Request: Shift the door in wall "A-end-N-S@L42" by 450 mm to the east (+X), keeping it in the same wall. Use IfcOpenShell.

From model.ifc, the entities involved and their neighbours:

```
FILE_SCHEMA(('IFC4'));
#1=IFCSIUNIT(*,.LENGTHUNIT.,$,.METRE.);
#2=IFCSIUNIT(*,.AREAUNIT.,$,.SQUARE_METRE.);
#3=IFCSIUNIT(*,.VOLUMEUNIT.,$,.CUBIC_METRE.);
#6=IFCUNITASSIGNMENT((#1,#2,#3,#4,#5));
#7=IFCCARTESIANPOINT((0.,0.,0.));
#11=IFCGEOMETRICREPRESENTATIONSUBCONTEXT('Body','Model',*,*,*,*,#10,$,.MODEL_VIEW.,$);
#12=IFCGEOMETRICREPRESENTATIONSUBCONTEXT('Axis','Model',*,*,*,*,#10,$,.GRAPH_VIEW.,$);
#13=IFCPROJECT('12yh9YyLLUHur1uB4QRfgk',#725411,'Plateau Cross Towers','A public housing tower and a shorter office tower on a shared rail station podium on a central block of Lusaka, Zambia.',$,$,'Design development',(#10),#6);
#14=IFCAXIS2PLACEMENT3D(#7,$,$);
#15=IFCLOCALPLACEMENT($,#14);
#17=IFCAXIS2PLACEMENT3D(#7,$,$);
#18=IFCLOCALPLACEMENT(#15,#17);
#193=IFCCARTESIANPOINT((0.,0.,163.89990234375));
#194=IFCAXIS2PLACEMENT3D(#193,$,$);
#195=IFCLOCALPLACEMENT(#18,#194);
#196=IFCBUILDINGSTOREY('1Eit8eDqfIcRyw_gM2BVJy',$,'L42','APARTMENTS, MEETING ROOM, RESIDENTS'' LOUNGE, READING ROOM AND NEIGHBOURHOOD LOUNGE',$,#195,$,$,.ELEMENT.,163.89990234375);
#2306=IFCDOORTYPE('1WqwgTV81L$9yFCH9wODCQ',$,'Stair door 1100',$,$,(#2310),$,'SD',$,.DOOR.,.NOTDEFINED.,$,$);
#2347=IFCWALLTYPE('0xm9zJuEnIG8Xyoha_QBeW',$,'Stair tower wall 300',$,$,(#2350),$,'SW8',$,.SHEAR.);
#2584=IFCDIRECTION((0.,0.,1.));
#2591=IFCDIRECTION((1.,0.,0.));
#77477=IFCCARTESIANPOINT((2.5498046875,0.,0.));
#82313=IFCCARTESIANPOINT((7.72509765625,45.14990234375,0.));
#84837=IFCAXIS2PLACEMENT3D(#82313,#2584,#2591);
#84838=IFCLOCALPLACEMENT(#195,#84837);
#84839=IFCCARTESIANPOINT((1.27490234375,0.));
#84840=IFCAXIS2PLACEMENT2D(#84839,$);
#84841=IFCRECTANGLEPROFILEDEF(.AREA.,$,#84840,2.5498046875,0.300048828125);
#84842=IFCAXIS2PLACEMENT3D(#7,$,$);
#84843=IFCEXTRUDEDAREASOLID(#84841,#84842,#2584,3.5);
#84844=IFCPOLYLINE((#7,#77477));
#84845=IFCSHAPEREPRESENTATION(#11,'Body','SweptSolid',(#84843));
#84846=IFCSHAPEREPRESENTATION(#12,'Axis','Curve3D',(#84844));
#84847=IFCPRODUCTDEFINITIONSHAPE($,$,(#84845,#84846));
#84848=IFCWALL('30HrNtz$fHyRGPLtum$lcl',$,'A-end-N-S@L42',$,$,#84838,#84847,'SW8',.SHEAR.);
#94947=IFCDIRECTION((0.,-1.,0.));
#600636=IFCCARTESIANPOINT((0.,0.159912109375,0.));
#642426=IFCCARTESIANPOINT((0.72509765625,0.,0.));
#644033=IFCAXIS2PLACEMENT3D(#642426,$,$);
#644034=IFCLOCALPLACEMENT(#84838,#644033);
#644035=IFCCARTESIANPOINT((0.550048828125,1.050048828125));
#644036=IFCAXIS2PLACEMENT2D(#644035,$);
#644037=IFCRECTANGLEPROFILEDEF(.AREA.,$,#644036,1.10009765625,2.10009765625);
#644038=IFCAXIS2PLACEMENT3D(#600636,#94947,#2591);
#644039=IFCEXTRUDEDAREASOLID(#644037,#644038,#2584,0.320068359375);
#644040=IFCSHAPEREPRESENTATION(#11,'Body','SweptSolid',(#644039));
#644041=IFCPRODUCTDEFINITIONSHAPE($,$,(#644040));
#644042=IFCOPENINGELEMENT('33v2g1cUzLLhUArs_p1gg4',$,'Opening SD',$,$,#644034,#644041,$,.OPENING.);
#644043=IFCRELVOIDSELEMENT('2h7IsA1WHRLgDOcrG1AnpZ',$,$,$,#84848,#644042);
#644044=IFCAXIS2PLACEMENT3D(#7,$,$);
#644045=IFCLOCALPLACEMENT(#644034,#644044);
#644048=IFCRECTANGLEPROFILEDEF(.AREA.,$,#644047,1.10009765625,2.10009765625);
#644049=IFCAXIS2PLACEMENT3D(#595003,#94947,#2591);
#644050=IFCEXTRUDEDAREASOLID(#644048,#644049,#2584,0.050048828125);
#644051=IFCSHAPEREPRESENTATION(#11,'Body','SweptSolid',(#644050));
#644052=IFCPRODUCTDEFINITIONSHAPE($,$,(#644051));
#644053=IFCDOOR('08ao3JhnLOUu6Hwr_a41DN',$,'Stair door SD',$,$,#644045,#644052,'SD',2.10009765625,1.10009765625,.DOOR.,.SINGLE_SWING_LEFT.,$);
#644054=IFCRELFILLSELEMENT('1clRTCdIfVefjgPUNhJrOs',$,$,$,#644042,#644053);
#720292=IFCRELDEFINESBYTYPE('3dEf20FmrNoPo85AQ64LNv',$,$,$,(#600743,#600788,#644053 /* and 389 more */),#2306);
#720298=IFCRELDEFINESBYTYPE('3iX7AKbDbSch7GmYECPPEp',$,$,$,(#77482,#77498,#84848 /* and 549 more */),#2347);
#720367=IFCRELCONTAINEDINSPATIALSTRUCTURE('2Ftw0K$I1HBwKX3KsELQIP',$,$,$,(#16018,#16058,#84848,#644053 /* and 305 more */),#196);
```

```python
import ifcopenshell
import ifcopenshell.api.geometry
import ifcopenshell.util.placement
import ifcopenshell.util.unit

model = ifcopenshell.open("model.ifc")
unit_scale = ifcopenshell.util.unit.calculate_unit_scale(model)

door = model.by_guid("08ao3JhnLOUu6Hwr_a41DN")
opening = door.FillsVoids[0].RelatingOpeningElement
wall = opening.VoidsElements[0].RelatingBuildingElement

wall_matrix = ifcopenshell.util.placement.get_local_placement(wall.ObjectPlacement)
shift = wall_matrix[:3, 0] * 0.45 / unit_scale
before = ifcopenshell.util.placement.get_local_placement(door.ObjectPlacement)[:3, 3].copy()

# The door is placed relative to its opening, so it follows when the opening moves.
matrix = ifcopenshell.util.placement.get_local_placement(opening.ObjectPlacement)
matrix[:3, 3] += shift
ifcopenshell.api.geometry.edit_object_placement(
    model, product=opening, matrix=matrix, is_si=False, should_transform_children=True
)

after = ifcopenshell.util.placement.get_local_placement(door.ObjectPlacement)[:3, 3]
print("door moved by", (after - before).round(3) + 0.0)

model.write("model_updated.ifc")
```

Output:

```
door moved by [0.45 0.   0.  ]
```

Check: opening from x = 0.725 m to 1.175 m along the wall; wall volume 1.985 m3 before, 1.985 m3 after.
